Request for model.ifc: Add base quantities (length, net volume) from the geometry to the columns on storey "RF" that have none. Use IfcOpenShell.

First a look at what the model holds.

```python
import ifcopenshell
import ifcopenshell.util.element
import ifcopenshell.util.unit

model = ifcopenshell.open("model.ifc")
print(model.schema)
for unit_type in ("LENGTHUNIT", "AREAUNIT", "VOLUMEUNIT"):
    print(unit_type, ifcopenshell.util.unit.calculate_unit_scale(model, unit_type))
storey = next(s for s in model.by_type("IfcBuildingStorey") if s.Name == "RF")
columns = [e for e in ifcopenshell.util.element.get_decomposition(storey) if e.is_a("IfcColumn")]
for e in sorted(columns, key=lambda e: e.id()):
    print(e.id(), e.is_a(), e.Name, list(ifcopenshell.util.element.get_psets(e, qtos_only=True)), sep=" | ")
```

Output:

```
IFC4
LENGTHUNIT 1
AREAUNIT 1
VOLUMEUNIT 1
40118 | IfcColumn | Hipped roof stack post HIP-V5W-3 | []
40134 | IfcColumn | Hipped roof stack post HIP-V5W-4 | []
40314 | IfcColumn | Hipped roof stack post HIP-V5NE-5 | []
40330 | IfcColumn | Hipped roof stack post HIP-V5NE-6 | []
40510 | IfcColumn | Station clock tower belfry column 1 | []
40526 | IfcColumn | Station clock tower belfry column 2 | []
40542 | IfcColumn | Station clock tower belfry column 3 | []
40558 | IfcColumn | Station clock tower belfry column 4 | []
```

```python
import ifcopenshell
import ifcopenshell.api.pset
import ifcopenshell.geom
import ifcopenshell.util.element
import ifcopenshell.util.shape
import ifcopenshell.util.unit

model = ifcopenshell.open("model.ifc")
unit_scale = ifcopenshell.util.unit.calculate_unit_scale(model)
volume_scale = ifcopenshell.util.unit.calculate_unit_scale(model, "VOLUMEUNIT")
settings = ifcopenshell.geom.settings()

storey = next(s for s in model.by_type("IfcBuildingStorey") if s.Name == "RF")
columns = [e for e in ifcopenshell.util.element.get_decomposition(storey) if e.is_a("IfcColumn")]

for e in sorted(columns, key=lambda e: e.id()):
    if ifcopenshell.util.element.get_psets(e, qtos_only=True, should_inherit=False):
        continue
    # Geometry comes back in metres, in the element's own axes.
    shape = ifcopenshell.geom.create_shape(settings, e)
    values = {
        "Length": ifcopenshell.util.shape.get_z(shape.geometry) / unit_scale,
        "NetVolume": ifcopenshell.util.shape.get_volume(shape.geometry) / volume_scale,
    }
    qto = ifcopenshell.api.pset.add_qto(model, product=e, name="Qto_ColumnBaseQuantities")
    ifcopenshell.api.pset.edit_qto(model, qto=qto, properties=values)
    print(e.id(), {k: round(v, 3) for k, v in values.items()})

model.write("model-out.ifc")
```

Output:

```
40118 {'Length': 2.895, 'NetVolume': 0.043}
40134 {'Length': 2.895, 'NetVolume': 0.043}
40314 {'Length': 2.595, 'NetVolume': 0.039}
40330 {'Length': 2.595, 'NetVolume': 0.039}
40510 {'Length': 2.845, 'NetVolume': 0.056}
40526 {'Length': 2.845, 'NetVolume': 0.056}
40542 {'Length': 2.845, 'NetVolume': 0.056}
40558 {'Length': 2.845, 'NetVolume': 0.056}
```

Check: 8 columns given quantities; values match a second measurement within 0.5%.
